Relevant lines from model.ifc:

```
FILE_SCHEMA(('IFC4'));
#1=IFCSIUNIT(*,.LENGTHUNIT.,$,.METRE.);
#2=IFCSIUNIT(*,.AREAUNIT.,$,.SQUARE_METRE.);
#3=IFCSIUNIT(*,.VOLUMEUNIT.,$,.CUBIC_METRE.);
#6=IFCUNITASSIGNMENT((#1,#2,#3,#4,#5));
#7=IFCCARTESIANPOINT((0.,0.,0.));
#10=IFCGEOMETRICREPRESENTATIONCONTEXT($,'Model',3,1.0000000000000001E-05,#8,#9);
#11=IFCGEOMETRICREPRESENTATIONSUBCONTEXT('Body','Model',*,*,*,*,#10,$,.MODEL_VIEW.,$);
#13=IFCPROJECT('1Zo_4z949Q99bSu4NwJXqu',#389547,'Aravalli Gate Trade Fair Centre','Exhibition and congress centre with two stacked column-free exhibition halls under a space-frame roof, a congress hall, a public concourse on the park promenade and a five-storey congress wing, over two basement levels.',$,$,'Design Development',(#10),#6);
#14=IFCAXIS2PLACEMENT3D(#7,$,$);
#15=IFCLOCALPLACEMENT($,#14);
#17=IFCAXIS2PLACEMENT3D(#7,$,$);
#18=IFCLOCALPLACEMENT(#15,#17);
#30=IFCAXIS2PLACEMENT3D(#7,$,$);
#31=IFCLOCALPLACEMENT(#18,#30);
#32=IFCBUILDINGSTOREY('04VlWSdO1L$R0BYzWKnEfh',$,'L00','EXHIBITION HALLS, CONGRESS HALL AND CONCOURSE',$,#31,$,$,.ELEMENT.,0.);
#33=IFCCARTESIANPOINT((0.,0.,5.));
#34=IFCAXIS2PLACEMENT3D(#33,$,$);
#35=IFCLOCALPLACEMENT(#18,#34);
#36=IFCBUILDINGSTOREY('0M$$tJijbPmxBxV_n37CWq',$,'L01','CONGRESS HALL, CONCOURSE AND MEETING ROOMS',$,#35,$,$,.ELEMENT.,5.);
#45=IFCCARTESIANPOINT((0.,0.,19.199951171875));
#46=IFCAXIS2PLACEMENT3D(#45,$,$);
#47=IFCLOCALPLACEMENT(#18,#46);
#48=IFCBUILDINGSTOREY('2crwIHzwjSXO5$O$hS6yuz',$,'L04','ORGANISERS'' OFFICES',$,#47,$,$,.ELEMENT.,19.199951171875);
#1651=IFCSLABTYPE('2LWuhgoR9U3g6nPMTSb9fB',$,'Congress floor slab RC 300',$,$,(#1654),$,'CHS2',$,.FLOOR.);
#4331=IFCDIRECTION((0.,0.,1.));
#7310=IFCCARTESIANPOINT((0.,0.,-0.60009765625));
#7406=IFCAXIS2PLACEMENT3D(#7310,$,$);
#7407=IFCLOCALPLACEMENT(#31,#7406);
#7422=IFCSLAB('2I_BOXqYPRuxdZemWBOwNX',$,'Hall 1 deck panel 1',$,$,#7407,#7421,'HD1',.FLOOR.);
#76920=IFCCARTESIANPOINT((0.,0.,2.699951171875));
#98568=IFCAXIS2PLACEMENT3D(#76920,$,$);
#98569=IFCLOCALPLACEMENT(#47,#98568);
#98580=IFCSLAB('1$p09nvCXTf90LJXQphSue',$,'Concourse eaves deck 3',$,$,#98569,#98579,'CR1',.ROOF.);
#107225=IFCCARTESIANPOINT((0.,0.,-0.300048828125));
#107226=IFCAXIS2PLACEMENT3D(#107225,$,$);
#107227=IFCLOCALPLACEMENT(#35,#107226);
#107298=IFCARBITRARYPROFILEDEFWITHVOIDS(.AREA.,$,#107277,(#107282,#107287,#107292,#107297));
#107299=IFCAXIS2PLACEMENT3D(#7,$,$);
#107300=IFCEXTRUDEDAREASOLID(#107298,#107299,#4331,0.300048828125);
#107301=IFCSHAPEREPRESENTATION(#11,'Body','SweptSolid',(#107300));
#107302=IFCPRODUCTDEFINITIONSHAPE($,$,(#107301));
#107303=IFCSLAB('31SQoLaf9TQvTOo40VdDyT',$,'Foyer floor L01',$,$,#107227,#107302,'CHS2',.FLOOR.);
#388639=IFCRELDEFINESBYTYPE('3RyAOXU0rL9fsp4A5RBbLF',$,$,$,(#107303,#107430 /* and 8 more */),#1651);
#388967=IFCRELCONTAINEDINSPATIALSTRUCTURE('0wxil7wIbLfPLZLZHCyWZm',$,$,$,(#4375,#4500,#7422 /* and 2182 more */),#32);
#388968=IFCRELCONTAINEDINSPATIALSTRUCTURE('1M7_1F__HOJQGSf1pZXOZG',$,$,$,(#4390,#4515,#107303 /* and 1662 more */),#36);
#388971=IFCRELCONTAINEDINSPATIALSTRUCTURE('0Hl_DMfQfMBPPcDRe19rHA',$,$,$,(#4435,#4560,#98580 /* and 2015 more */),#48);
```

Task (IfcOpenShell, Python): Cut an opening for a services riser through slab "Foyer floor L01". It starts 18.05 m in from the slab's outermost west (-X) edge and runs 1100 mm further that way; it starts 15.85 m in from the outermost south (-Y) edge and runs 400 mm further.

```python
import numpy as np
import ifcopenshell
import ifcopenshell.api.feature
import ifcopenshell.api.geometry
import ifcopenshell.api.root
import ifcopenshell.geom
import ifcopenshell.util.placement
import ifcopenshell.util.representation
import ifcopenshell.util.shape
import ifcopenshell.util.unit

model = ifcopenshell.open("model.ifc")
unit_scale = ifcopenshell.util.unit.calculate_unit_scale(model)
settings = ifcopenshell.geom.settings()


def volume(element):
    """Net volume in cubic metres, openings subtracted."""
    shape = ifcopenshell.geom.create_shape(settings, element)
    return ifcopenshell.util.shape.get_volume(shape.geometry)


slab = model.by_guid("31SQoLaf9TQvTOo40VdDyT")
before = volume(slab)

# Extent in the slab's own axes, in metres. The edges named are its -X and -Y sides.
slab_shape = ifcopenshell.geom.create_shape(settings, slab)
vertices = ifcopenshell.util.shape.get_vertices(slab_shape.geometry)
x_min, y_min, bottom = vertices.min(axis=0)
top = vertices[:, 2].max()

opening = ifcopenshell.api.root.create_entity(model, ifc_class="IfcOpeningElement", name="Services riser opening", predefined_type="OPENING")
context = ifcopenshell.util.representation.get_context(model, "Model", "Body", "MODEL_VIEW")
width, depth = 1.1, 0.4
outline = [(0.0, 0.0), (width, 0.0), (width, depth), (0.0, depth), (0.0, 0.0)]
# Overshoot both faces by 50 mm so the cut is clean.
shape = ifcopenshell.api.geometry.add_slab_representation(
    model, context=context, depth=top - bottom + 0.1, polyline=outline
)
ifcopenshell.api.geometry.assign_representation(model, product=opening, representation=shape)

matrix = ifcopenshell.util.placement.get_local_placement(slab.ObjectPlacement)
matrix[:, 3] = matrix @ np.append(np.array([x_min + 18.05, y_min + 15.85, bottom - 0.05]) / unit_scale, 1.0)
ifcopenshell.api.geometry.edit_object_placement(model, product=opening, matrix=matrix, is_si=False)
ifcopenshell.api.feature.add_feature(model, feature=opening, element=slab)

after = volume(slab)

print(f"slab volume {before:.3f} -> {after:.3f} m3")

model.write("model_edited.ifc")
```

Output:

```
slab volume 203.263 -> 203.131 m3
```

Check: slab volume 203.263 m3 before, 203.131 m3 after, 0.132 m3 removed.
